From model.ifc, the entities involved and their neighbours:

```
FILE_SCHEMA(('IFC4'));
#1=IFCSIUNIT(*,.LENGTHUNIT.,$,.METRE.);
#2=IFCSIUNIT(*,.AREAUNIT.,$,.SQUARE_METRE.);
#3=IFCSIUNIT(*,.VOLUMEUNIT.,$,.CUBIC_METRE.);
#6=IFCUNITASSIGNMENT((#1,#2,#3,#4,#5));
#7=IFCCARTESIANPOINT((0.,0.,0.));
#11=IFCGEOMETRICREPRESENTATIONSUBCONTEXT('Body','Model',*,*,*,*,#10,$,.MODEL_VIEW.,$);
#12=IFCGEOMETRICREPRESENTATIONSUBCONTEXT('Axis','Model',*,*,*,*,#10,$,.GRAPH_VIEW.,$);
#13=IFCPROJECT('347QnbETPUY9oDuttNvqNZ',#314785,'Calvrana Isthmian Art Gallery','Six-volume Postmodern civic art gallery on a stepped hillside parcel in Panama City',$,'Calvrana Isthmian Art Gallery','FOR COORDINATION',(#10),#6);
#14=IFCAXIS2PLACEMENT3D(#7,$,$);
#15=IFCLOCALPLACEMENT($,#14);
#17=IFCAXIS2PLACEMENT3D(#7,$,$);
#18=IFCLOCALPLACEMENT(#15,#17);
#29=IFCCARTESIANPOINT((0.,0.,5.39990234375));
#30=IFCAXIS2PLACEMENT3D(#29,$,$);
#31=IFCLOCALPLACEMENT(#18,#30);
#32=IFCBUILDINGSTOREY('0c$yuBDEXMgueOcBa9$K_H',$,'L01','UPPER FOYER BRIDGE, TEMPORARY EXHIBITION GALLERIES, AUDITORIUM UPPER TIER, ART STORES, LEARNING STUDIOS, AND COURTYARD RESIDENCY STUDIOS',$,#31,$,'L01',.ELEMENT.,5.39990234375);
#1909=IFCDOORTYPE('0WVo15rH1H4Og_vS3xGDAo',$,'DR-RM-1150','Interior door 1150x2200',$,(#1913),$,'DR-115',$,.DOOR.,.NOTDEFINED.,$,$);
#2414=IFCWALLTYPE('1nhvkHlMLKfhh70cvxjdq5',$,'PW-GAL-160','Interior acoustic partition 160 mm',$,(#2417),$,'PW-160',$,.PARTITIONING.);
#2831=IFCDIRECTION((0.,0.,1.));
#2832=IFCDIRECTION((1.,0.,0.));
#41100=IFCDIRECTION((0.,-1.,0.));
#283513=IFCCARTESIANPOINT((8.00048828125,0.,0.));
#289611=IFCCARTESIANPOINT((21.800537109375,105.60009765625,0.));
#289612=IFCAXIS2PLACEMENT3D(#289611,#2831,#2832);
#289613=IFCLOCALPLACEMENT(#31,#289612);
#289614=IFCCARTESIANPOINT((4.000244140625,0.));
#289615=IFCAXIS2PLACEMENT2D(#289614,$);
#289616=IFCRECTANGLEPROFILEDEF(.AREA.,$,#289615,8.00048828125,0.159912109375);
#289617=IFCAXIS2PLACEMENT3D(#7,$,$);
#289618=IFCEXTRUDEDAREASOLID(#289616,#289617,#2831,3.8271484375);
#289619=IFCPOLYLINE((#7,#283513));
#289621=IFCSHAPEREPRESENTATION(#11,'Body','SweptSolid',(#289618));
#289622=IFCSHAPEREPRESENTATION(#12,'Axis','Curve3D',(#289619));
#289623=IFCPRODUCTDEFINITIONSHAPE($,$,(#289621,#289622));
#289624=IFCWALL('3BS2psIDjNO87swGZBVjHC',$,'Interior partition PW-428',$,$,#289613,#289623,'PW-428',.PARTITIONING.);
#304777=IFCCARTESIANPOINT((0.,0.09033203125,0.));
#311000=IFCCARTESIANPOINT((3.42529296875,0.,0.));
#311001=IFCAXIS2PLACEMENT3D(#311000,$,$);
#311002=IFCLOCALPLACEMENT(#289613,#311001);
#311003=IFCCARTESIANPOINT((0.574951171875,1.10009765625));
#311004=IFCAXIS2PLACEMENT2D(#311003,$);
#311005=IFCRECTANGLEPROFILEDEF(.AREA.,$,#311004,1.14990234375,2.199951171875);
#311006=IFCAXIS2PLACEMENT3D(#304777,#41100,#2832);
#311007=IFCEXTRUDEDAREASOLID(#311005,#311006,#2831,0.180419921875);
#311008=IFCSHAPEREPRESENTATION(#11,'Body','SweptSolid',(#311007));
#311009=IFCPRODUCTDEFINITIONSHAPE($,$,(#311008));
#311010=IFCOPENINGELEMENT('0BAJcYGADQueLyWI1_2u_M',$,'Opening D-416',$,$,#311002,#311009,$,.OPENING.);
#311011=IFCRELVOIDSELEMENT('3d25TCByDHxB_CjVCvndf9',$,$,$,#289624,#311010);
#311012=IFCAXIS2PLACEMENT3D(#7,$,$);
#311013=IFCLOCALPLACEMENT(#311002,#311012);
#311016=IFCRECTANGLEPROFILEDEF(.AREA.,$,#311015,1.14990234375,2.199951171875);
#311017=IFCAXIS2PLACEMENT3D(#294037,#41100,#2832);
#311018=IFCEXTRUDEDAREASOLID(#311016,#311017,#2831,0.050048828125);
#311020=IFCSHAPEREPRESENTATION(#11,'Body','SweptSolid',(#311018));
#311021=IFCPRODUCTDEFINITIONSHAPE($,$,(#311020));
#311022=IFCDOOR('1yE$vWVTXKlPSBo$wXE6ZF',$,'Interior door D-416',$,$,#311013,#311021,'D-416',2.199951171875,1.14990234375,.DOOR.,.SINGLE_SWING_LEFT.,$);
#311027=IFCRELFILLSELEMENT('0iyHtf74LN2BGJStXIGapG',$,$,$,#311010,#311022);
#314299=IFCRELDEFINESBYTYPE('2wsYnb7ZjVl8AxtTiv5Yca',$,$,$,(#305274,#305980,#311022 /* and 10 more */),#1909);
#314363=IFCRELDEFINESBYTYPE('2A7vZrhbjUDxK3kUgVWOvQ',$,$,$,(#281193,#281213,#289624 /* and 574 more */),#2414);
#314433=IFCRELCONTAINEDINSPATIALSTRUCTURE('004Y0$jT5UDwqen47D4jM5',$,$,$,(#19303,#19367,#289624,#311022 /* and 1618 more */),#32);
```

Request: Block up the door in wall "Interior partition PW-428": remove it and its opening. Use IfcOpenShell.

```python
import ifcopenshell
import ifcopenshell.api.feature
import ifcopenshell.api.root
import ifcopenshell.geom
import ifcopenshell.util.shape

model = ifcopenshell.open("model.ifc")
settings = ifcopenshell.geom.settings()


def volume(element):
    """Net volume in cubic metres, openings subtracted."""
    shape = ifcopenshell.geom.create_shape(settings, element)
    return ifcopenshell.util.shape.get_volume(shape.geometry)


door = model.by_guid("1yE$vWVTXKlPSBo$wXE6ZF")
opening = door.FillsVoids[0].RelatingOpeningElement
wall = opening.VoidsElements[0].RelatingBuildingElement
before = volume(wall)

ifcopenshell.api.root.remove_product(model, product=door)
ifcopenshell.api.feature.remove_feature(model, feature=opening)

after = volume(wall)

print(f"wall volume {before:.3f} -> {after:.3f} m3")

model.write("model_v2.ifc")
```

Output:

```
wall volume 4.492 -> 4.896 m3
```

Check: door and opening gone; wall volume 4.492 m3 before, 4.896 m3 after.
